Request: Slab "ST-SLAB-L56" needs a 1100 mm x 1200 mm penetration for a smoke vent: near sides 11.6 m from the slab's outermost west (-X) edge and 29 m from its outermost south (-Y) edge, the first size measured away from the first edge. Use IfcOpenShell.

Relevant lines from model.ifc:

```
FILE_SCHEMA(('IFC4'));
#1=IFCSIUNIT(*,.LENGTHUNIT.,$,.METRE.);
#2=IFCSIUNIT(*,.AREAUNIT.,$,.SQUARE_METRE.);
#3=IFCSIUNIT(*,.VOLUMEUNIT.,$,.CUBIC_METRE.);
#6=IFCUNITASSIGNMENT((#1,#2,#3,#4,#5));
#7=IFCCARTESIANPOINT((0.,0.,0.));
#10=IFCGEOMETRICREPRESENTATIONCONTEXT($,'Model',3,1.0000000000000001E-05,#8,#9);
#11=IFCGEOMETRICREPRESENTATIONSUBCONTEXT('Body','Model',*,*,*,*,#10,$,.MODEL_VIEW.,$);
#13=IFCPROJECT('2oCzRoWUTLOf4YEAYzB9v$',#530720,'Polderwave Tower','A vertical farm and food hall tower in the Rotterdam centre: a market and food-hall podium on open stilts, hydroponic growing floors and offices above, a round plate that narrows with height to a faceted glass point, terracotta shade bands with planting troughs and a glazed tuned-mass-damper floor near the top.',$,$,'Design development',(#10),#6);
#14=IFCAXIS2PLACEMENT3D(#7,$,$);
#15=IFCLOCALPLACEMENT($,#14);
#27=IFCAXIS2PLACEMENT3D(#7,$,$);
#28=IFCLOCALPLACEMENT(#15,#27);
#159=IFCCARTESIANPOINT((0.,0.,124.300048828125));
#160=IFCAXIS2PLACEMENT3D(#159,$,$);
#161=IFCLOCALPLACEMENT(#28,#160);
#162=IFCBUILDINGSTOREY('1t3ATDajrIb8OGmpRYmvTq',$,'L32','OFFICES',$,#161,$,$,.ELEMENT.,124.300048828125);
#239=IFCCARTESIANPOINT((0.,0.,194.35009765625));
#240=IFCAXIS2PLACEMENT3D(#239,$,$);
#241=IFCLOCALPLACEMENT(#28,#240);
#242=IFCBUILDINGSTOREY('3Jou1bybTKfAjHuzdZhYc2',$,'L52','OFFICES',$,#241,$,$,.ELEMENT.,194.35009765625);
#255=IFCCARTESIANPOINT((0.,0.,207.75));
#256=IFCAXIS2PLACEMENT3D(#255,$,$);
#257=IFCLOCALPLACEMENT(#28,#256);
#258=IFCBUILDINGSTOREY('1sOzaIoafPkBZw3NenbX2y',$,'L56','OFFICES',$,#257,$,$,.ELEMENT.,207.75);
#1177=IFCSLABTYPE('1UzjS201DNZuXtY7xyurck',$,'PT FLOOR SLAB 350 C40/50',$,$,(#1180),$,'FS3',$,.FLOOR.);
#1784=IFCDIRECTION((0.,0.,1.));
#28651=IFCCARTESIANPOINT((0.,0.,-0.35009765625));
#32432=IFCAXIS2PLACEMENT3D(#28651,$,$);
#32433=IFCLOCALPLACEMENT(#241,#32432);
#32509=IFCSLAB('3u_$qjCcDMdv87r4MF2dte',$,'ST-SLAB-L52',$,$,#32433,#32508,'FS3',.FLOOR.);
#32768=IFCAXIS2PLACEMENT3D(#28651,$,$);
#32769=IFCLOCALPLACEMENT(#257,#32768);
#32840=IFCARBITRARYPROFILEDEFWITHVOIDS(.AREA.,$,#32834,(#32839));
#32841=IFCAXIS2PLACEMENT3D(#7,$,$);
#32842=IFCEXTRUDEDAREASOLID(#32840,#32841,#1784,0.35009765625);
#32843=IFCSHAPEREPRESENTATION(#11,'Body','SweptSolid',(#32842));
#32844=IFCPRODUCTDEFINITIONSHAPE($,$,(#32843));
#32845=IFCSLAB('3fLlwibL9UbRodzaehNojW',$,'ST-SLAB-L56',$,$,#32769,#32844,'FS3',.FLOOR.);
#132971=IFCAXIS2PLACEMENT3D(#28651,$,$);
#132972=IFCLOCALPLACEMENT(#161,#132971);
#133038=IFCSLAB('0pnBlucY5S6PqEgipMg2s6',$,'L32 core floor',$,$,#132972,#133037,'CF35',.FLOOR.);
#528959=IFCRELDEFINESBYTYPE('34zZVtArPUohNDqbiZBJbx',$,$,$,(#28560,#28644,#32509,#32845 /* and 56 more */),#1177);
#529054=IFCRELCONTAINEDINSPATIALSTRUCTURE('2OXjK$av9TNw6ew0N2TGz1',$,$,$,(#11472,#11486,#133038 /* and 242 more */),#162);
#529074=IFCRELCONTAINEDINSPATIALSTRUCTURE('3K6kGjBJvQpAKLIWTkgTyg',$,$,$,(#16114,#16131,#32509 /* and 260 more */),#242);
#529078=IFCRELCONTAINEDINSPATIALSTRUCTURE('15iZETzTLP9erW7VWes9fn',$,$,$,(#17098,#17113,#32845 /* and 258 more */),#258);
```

```python
import numpy as np
import ifcopenshell
import ifcopenshell.api.feature
import ifcopenshell.api.geometry
import ifcopenshell.api.root
import ifcopenshell.geom
import ifcopenshell.util.placement
import ifcopenshell.util.representation
import ifcopenshell.util.shape
import ifcopenshell.util.unit

model = ifcopenshell.open("model.ifc")
unit_scale = ifcopenshell.util.unit.calculate_unit_scale(model)
settings = ifcopenshell.geom.settings()


def volume(element):
    """Net volume in cubic metres, openings subtracted."""
    shape = ifcopenshell.geom.create_shape(settings, element)
    return ifcopenshell.util.shape.get_volume(shape.geometry)


slab = model.by_id(32845)
before = volume(slab)

# Extent in the slab's own axes, in metres. The edges named are its -X and -Y sides.
slab_shape = ifcopenshell.geom.create_shape(settings, slab)
vertices = ifcopenshell.util.shape.get_vertices(slab_shape.geometry)
x_min, y_min, bottom = vertices.min(axis=0)
top = vertices[:, 2].max()

opening = ifcopenshell.api.root.create_entity(model, ifc_class="IfcOpeningElement", name="Smoke vent opening", predefined_type="OPENING")
context = ifcopenshell.util.representation.get_context(model, "Model", "Body", "MODEL_VIEW")
width, depth = 1.1, 1.2
outline = [(0.0, 0.0), (width, 0.0), (width, depth), (0.0, depth), (0.0, 0.0)]
# Overshoot both faces by 50 mm so the cut is clean.
shape = ifcopenshell.api.geometry.add_slab_representation(
    model, context=context, depth=top - bottom + 0.1, polyline=outline
)
ifcopenshell.api.geometry.assign_representation(model, product=opening, representation=shape)

matrix = ifcopenshell.util.placement.get_local_placement(slab.ObjectPlacement)
matrix[:, 3] = matrix @ np.append(np.array([x_min + 11.6, y_min + 29, bottom - 0.05]) / unit_scale, 1.0)
ifcopenshell.api.geometry.edit_object_placement(model, product=opening, matrix=matrix, is_si=False)
ifcopenshell.api.feature.add_feature(model, feature=opening, element=slab)

after = volume(slab)

print(f"slab volume {before:.3f} -> {after:.3f} m3")

model.write("model-out.ifc")
```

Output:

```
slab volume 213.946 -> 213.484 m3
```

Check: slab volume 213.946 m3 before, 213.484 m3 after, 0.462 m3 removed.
